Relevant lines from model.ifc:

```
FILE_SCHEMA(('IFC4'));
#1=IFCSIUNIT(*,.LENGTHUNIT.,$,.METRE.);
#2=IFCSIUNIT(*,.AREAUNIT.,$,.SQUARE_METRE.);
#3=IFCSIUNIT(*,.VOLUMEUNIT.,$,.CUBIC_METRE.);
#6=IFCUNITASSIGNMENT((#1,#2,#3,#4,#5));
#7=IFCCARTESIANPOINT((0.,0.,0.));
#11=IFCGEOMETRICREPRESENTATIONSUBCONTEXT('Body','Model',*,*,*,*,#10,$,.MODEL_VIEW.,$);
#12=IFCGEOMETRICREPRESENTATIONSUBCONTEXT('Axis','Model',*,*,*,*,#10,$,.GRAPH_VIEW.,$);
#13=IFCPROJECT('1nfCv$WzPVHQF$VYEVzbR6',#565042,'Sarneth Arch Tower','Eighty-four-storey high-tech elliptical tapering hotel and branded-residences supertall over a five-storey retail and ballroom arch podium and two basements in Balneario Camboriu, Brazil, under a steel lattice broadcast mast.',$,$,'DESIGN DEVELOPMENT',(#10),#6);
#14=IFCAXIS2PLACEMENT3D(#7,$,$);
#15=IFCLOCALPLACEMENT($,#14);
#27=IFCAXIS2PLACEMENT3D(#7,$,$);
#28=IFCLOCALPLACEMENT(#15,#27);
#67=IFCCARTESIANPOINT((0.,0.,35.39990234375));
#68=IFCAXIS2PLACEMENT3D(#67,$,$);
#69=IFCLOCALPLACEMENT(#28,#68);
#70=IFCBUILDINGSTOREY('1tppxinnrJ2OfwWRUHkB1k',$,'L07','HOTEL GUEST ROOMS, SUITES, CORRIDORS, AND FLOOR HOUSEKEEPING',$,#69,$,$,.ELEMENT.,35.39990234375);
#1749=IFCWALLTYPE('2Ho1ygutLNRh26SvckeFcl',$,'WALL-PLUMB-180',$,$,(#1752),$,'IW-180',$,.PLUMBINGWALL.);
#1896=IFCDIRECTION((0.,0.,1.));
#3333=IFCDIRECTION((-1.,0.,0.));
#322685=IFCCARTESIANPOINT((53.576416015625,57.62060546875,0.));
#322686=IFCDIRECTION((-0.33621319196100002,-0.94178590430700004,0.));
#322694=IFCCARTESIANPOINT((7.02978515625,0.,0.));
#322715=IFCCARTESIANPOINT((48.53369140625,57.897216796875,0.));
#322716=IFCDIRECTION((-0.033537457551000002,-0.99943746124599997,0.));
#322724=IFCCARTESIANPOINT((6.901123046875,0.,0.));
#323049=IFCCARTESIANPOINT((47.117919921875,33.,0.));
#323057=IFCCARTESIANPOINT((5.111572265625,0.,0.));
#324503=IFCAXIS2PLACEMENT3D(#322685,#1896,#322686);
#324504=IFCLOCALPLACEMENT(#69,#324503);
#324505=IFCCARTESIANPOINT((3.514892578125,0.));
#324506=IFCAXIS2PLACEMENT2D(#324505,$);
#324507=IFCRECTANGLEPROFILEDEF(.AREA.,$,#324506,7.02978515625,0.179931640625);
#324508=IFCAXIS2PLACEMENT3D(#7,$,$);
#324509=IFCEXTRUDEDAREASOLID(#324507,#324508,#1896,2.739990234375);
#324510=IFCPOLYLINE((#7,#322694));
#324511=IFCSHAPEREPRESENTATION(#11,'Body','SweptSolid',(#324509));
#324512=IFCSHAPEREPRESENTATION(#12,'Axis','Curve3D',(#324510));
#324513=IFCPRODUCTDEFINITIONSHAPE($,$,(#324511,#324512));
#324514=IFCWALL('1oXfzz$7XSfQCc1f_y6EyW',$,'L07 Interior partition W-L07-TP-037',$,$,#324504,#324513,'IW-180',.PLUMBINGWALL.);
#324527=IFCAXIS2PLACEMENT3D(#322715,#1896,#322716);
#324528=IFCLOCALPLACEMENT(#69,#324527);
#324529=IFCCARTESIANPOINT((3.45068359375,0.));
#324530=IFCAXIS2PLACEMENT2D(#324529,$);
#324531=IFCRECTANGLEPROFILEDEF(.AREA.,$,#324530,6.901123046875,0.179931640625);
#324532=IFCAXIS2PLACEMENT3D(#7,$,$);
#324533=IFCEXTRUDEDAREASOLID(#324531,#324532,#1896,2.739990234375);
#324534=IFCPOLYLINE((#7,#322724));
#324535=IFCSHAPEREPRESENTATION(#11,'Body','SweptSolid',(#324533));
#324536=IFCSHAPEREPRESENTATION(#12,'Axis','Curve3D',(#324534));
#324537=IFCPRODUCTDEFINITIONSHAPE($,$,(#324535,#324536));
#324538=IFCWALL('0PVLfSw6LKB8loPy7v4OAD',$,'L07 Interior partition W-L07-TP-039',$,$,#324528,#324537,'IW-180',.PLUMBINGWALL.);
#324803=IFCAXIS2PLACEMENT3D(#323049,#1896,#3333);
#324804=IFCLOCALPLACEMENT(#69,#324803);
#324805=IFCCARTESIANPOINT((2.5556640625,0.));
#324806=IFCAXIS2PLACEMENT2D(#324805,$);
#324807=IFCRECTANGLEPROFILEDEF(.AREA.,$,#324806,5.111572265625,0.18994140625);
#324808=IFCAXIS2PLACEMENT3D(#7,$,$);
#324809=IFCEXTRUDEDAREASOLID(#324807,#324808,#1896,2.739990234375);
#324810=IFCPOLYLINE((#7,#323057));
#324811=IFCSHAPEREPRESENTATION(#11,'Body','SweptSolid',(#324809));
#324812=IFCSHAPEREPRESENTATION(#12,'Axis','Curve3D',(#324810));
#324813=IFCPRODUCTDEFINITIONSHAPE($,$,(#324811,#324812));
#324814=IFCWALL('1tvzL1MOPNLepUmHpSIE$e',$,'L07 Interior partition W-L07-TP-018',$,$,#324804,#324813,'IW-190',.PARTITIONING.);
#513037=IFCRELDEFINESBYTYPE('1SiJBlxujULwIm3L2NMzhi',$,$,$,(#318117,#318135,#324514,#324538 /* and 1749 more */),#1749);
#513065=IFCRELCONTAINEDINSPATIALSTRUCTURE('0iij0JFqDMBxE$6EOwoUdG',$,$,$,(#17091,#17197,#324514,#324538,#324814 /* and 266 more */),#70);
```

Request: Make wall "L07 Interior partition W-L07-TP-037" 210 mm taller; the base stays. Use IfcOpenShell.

```python
import ifcopenshell
import ifcopenshell.geom
import ifcopenshell.util.representation
import ifcopenshell.util.shape
import ifcopenshell.util.unit

model = ifcopenshell.open("model.ifc")
unit_scale = ifcopenshell.util.unit.calculate_unit_scale(model)
settings = ifcopenshell.geom.settings()


def volume(element):
    """Net volume in cubic metres, openings subtracted."""
    shape = ifcopenshell.geom.create_shape(settings, element)
    return ifcopenshell.util.shape.get_volume(shape.geometry)


wall = model.by_id(324514)
before = volume(wall)

body = ifcopenshell.util.representation.get_representation(wall, "Model", "Body")
solid = body.Items[0]
old_height = solid.Depth
solid.Depth += 0.21 / unit_scale
after = volume(wall)

print(f"height {old_height:g} -> {solid.Depth:g}, volume {before:.3f} -> {after:.3f} m3")

model.write("model_v2.ifc")
```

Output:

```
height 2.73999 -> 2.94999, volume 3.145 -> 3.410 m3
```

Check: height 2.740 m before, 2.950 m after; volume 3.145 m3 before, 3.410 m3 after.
